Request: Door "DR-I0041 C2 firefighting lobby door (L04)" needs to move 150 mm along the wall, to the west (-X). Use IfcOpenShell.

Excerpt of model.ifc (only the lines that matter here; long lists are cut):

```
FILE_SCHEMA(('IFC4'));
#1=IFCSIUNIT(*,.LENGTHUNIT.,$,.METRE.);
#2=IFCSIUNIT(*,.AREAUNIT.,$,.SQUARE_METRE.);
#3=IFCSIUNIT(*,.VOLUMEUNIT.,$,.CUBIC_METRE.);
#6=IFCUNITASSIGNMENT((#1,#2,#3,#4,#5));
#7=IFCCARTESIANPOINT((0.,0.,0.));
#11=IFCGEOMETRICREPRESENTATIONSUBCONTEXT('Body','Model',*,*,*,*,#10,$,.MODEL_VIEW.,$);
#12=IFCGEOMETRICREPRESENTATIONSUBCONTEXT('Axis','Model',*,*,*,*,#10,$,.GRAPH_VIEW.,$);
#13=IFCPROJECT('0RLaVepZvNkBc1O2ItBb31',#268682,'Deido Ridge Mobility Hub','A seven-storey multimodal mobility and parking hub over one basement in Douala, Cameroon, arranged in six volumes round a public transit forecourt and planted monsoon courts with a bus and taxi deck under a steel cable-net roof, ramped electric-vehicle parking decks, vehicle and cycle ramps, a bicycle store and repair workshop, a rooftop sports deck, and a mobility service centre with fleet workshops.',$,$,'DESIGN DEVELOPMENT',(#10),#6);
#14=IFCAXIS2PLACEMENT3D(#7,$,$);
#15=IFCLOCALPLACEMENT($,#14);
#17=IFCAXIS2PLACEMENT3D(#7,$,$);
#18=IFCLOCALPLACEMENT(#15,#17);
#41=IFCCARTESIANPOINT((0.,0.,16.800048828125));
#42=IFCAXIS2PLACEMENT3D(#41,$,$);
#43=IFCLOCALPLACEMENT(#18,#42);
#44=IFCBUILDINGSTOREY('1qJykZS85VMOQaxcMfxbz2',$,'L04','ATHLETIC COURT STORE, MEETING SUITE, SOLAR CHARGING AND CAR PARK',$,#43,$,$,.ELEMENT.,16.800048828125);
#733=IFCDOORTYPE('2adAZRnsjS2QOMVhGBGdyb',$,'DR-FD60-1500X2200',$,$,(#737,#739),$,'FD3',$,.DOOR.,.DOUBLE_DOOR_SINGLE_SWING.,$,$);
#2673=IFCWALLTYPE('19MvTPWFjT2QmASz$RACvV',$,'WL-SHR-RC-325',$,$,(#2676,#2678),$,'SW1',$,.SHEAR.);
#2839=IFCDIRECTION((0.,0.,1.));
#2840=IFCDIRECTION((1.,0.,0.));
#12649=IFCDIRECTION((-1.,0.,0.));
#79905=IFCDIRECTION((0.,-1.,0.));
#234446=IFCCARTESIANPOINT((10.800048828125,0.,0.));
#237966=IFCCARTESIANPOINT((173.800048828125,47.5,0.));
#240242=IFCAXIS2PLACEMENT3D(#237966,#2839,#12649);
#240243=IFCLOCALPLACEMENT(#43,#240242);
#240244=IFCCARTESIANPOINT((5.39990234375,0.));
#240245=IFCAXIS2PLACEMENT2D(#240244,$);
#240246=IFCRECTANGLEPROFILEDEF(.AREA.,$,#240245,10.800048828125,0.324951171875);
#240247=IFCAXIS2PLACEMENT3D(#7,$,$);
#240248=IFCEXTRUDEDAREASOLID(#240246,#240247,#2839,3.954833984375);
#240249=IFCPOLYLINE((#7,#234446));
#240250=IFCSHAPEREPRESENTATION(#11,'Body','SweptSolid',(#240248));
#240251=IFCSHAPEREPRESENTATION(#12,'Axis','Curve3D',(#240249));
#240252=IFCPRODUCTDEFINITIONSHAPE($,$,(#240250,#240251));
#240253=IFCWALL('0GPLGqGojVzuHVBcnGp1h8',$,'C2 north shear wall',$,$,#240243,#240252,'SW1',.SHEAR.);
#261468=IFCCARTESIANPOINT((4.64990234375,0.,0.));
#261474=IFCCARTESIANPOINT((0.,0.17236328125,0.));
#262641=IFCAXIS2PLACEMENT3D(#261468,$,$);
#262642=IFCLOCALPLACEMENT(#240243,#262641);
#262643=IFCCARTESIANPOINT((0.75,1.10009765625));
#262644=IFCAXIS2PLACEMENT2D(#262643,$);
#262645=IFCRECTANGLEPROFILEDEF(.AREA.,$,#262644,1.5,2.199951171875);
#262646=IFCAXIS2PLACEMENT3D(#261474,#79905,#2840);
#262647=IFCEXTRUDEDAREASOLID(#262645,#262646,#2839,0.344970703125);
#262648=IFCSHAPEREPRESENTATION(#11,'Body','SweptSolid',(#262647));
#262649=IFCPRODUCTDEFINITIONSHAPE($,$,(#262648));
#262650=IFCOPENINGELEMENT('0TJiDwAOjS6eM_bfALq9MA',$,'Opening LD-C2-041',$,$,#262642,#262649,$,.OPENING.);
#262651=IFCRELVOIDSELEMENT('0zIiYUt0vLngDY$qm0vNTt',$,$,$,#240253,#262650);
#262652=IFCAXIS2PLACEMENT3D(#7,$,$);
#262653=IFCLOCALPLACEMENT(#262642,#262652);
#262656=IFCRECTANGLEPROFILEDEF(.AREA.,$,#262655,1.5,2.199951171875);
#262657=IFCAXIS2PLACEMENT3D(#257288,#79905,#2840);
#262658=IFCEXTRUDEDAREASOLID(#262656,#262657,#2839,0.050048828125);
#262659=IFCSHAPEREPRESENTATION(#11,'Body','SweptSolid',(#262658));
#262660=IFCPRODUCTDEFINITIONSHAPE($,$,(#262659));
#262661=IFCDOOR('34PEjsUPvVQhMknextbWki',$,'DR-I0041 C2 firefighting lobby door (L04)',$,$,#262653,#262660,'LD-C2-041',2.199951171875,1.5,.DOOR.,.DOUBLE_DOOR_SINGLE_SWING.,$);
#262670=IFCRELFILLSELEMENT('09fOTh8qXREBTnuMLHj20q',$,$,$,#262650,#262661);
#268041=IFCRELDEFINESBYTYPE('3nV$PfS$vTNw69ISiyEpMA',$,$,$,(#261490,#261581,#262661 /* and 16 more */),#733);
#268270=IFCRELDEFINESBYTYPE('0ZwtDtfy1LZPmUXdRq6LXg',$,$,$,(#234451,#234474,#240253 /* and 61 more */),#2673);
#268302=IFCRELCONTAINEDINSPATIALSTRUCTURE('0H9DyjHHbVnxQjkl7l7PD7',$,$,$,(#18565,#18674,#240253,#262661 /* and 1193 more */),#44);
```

```python
import ifcopenshell
import ifcopenshell.api.geometry
import ifcopenshell.util.placement

model = ifcopenshell.open("model.ifc")

door = model.by_guid("34PEjsUPvVQhMknextbWki")
opening = door.FillsVoids[0].RelatingOpeningElement
wall = opening.VoidsElements[0].RelatingBuildingElement

wall_matrix = ifcopenshell.util.placement.get_local_placement(wall.ObjectPlacement)
shift = wall_matrix[:3, 0] * 0.15
before = ifcopenshell.util.placement.get_local_placement(door.ObjectPlacement)[:3, 3].copy()

# The door is placed relative to its opening, so it follows when the opening moves.
matrix = ifcopenshell.util.placement.get_local_placement(opening.ObjectPlacement)
matrix[:3, 3] += shift
ifcopenshell.api.geometry.edit_object_placement(
    model, product=opening, matrix=matrix, is_si=False, should_transform_children=True
)

after = ifcopenshell.util.placement.get_local_placement(door.ObjectPlacement)[:3, 3]
print("door moved by", (after - before).round(3) + 0.0)

model.write("model_v2.ifc")
```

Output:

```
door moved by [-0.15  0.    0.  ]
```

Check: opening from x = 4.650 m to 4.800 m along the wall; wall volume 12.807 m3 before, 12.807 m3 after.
